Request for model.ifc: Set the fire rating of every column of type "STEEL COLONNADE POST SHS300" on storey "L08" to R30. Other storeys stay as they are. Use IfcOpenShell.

First a look at what the model holds.

```python
import ifcopenshell
import ifcopenshell.util.element

model = ifcopenshell.open("model.ifc")
print(model.schema)
storey = next(s for s in model.by_type("IfcBuildingStorey") if s.Name == "L08")
columns = [e for e in ifcopenshell.util.element.get_decomposition(storey) if e.is_a("IfcColumn")]
seen = {}
for e in columns:
    element_type = ifcopenshell.util.element.get_type(e)
    key = (element_type.Name if element_type != e and element_type else None, ifcopenshell.util.element.get_pset(e, "Pset_ColumnCommon", "FireRating"))
    seen[key] = seen.get(key, 0) + 1
for (name, value), count in sorted(seen.items(), key=str):
    print(count, "x", name, "|", value)
```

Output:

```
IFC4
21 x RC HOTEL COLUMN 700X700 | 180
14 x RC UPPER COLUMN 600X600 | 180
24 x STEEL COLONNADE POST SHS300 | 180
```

```python
import ifcopenshell
import ifcopenshell.api.pset
import ifcopenshell.util.element

model = ifcopenshell.open("model.ifc")

storey = next(s for s in model.by_type("IfcBuildingStorey") if s.Name == "L08")
columns = [e for e in ifcopenshell.util.element.get_decomposition(storey) if e.is_a("IfcColumn")]

count = 0
for e in columns:
    element_type = ifcopenshell.util.element.get_type(e)
    if element_type in (None, e) or element_type.Name != "STEEL COLONNADE POST SHS300":
        continue
    # add_pset returns the element's existing set when there is one.
    pset = ifcopenshell.api.pset.add_pset(model, product=e, name="Pset_ColumnCommon")
    ifcopenshell.api.pset.edit_pset(model, pset=pset, properties={"FireRating": "R30"})
    count += 1

print(count, "columns updated")

model.write("model_v2.ifc")
```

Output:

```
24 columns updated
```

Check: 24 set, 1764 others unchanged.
